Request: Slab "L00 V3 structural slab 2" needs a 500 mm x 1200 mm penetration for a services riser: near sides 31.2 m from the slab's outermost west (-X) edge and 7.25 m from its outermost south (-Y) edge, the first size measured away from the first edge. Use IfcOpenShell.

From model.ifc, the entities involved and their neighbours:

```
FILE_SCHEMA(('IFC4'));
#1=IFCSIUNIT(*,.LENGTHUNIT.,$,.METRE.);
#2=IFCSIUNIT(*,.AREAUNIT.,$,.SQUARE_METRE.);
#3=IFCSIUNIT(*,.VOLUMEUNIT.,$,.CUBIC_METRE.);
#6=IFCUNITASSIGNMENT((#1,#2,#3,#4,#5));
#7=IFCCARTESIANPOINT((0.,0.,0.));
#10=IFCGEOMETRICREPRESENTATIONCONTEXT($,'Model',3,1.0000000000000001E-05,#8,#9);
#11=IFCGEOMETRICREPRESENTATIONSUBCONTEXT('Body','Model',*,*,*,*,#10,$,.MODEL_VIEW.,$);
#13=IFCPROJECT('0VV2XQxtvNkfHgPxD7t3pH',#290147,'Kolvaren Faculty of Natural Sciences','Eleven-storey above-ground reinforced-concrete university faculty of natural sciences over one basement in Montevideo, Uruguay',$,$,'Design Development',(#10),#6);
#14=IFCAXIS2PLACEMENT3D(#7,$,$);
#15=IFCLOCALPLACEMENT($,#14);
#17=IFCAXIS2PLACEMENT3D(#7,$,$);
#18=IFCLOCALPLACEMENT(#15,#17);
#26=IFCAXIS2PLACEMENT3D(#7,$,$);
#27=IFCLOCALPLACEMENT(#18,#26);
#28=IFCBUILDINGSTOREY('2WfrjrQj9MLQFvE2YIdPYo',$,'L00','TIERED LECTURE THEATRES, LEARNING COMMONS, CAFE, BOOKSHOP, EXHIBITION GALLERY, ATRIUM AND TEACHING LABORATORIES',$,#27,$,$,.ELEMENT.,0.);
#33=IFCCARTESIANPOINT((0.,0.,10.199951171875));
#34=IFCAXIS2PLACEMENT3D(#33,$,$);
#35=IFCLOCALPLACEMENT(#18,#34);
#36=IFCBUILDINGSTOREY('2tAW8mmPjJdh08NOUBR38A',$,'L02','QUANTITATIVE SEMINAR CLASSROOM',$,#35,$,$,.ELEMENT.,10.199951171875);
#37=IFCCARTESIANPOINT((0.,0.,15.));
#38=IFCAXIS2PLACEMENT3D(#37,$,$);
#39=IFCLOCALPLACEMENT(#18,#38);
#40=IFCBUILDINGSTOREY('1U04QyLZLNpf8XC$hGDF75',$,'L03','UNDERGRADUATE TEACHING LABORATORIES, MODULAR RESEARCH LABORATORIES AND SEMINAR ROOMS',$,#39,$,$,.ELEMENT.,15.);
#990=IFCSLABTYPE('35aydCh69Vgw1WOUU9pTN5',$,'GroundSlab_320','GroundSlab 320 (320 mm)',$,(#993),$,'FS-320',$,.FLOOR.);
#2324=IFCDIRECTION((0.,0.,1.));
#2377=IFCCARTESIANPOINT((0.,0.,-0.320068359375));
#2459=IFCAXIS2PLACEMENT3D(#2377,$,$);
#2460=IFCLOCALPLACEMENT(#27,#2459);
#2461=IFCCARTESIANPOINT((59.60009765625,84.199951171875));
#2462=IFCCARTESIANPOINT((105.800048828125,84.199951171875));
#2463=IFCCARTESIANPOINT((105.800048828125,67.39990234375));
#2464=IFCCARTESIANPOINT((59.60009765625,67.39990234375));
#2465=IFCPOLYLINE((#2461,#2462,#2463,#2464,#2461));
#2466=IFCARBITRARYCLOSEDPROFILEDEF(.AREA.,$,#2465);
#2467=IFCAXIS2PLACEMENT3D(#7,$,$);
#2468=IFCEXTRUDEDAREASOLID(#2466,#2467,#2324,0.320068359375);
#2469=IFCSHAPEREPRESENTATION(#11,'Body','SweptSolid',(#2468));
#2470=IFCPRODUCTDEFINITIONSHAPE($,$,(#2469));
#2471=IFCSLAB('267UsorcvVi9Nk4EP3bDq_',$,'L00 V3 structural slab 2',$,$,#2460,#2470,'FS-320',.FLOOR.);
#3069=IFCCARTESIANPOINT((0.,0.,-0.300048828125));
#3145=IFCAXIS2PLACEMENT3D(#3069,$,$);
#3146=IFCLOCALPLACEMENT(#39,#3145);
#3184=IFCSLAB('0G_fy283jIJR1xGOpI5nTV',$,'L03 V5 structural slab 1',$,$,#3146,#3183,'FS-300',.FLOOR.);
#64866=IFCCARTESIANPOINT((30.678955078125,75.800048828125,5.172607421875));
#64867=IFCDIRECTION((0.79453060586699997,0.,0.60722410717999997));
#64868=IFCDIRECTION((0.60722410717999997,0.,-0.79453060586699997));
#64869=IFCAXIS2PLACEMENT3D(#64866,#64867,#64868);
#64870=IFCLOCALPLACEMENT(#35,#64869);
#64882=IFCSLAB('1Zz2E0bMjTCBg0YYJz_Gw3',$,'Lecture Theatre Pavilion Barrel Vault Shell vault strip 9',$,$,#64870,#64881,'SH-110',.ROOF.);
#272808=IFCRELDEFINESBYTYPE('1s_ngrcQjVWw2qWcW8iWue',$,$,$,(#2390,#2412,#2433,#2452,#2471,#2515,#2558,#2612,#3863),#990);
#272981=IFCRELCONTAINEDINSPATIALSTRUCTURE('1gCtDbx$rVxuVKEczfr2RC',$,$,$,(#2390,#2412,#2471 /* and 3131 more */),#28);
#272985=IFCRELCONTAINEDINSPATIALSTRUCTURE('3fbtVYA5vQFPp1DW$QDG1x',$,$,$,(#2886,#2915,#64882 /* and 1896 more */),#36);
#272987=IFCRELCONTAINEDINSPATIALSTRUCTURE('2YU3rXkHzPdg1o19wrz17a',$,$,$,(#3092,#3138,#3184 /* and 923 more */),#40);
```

```python
import numpy as np
import ifcopenshell
import ifcopenshell.api.feature
import ifcopenshell.api.geometry
import ifcopenshell.api.root
import ifcopenshell.geom
import ifcopenshell.util.placement
import ifcopenshell.util.representation
import ifcopenshell.util.shape
import ifcopenshell.util.unit

model = ifcopenshell.open("model.ifc")
unit_scale = ifcopenshell.util.unit.calculate_unit_scale(model)
settings = ifcopenshell.geom.settings()


def volume(element):
    """Net volume in cubic metres, openings subtracted."""
    shape = ifcopenshell.geom.create_shape(settings, element)
    return ifcopenshell.util.shape.get_volume(shape.geometry)


slab = model.by_id(2471)
before = volume(slab)

# Extent in the slab's own axes, in metres. The edges named are its -X and -Y sides.
slab_shape = ifcopenshell.geom.create_shape(settings, slab)
vertices = ifcopenshell.util.shape.get_vertices(slab_shape.geometry)
x_min, y_min, bottom = vertices.min(axis=0)
top = vertices[:, 2].max()

opening = ifcopenshell.api.root.create_entity(model, ifc_class="IfcOpeningElement", name="Services riser opening", predefined_type="OPENING")
context = ifcopenshell.util.representation.get_context(model, "Model", "Body", "MODEL_VIEW")
width, depth = 0.5, 1.2
outline = [(0.0, 0.0), (width, 0.0), (width, depth), (0.0, depth), (0.0, 0.0)]
# Overshoot both faces by 50 mm so the cut is clean.
shape = ifcopenshell.api.geometry.add_slab_representation(
    model, context=context, depth=top - bottom + 0.1, polyline=outline
)
ifcopenshell.api.geometry.assign_representation(model, product=opening, representation=shape)

matrix = ifcopenshell.util.placement.get_local_placement(slab.ObjectPlacement)
matrix[:, 3] = matrix @ np.append(np.array([x_min + 31.2, y_min + 7.25, bottom - 0.05]) / unit_scale, 1.0)
ifcopenshell.api.geometry.edit_object_placement(model, product=opening, matrix=matrix, is_si=False)
ifcopenshell.api.feature.add_feature(model, feature=opening, element=slab)

after = volume(slab)

print(f"slab volume {before:.3f} -> {after:.3f} m3")

model.write("model_updated.ifc")
```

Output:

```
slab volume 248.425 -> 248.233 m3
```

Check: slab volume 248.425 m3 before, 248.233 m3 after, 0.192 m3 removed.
